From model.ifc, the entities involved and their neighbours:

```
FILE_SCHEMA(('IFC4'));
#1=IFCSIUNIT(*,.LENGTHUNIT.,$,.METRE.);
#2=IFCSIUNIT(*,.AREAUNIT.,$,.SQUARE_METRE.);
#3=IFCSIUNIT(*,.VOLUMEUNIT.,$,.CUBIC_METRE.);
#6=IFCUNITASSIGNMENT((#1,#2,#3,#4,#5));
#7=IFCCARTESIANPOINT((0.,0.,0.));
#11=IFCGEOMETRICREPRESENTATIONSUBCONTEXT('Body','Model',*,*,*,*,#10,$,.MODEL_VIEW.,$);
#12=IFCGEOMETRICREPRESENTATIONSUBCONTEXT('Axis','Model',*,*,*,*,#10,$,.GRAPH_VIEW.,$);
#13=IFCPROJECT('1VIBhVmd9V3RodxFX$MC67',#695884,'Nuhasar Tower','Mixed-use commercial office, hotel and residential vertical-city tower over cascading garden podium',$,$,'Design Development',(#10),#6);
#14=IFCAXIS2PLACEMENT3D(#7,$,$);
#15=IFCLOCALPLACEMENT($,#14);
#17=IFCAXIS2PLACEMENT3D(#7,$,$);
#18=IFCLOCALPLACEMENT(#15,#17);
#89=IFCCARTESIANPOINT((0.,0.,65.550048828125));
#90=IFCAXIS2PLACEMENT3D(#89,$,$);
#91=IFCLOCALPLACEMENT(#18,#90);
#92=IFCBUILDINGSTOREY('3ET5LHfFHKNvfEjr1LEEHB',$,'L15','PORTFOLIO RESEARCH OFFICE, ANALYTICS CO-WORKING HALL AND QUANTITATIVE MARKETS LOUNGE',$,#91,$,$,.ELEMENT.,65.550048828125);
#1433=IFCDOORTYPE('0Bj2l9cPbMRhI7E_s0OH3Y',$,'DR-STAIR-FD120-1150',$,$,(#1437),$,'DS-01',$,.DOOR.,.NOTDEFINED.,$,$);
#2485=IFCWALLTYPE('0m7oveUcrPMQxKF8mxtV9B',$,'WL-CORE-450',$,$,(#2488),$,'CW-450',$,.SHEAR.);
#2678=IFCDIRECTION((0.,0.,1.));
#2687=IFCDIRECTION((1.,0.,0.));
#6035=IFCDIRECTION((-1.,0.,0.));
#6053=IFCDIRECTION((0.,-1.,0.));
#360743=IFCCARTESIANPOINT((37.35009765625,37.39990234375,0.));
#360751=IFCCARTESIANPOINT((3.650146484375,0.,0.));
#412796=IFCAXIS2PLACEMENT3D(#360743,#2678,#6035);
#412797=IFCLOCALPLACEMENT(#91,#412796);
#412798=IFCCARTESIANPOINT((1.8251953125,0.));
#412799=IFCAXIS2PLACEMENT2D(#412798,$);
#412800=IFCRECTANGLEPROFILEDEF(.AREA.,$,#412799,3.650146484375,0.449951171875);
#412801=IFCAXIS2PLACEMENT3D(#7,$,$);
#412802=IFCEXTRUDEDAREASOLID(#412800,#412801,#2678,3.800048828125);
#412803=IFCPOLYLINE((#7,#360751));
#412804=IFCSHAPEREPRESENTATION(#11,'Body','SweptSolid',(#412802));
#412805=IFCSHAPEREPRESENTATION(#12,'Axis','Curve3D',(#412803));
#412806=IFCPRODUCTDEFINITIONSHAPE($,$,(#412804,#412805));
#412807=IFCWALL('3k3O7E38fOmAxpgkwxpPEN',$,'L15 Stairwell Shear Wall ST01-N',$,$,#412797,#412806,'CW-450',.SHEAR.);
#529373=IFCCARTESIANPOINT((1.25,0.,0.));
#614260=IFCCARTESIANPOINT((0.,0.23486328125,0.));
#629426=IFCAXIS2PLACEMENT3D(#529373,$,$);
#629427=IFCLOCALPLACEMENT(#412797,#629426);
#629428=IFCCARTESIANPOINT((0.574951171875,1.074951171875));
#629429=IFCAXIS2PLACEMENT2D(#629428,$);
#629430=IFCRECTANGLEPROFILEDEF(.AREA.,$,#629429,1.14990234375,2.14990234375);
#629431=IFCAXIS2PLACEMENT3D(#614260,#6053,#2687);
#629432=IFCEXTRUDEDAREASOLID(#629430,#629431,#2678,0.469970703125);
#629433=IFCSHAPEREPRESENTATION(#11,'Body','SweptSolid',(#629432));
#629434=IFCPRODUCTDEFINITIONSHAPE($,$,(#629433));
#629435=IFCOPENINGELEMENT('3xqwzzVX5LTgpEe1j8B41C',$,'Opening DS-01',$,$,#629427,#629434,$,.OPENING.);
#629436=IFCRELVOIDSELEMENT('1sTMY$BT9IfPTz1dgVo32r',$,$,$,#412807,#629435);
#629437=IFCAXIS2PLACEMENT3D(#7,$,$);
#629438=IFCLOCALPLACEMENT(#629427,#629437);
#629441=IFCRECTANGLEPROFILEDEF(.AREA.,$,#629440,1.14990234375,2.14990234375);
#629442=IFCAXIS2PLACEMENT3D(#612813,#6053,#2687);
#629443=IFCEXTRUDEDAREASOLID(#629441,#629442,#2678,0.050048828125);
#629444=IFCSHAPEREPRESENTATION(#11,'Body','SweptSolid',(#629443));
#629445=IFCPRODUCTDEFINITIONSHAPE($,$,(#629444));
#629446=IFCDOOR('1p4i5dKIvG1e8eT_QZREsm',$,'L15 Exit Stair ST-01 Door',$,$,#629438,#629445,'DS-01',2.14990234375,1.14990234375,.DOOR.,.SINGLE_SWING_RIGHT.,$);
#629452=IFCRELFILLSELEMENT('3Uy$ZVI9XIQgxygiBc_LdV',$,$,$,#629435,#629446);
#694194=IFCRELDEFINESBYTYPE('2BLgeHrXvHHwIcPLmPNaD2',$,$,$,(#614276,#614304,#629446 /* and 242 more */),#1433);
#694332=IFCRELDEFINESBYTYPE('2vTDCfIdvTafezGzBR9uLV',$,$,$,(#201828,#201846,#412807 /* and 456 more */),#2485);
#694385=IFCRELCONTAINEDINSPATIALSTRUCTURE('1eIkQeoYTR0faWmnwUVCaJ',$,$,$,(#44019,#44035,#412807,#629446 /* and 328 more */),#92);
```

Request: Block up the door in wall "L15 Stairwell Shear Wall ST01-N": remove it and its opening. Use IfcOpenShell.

```python
import ifcopenshell
import ifcopenshell.api.feature
import ifcopenshell.api.root
import ifcopenshell.geom
import ifcopenshell.util.shape

model = ifcopenshell.open("model.ifc")
settings = ifcopenshell.geom.settings()


def volume(element):
    """Net volume in cubic metres, openings subtracted."""
    shape = ifcopenshell.geom.create_shape(settings, element)
    return ifcopenshell.util.shape.get_volume(shape.geometry)


door = model.by_id(629446)
opening = door.FillsVoids[0].RelatingOpeningElement
wall = opening.VoidsElements[0].RelatingBuildingElement
before = volume(wall)

ifcopenshell.api.root.remove_product(model, product=door)
ifcopenshell.api.feature.remove_feature(model, feature=opening)

after = volume(wall)

print(f"wall volume {before:.3f} -> {after:.3f} m3")

model.write("model_edited.ifc")
```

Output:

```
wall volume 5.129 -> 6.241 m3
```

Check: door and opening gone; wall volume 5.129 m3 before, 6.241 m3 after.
